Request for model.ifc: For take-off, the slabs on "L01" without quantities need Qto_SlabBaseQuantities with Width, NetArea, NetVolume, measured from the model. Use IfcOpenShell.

First a look at what the model holds.

```python
import ifcopenshell
import ifcopenshell.util.element
import ifcopenshell.util.unit

model = ifcopenshell.open("model.ifc")
print(model.schema)
for unit_type in ("LENGTHUNIT", "AREAUNIT", "VOLUMEUNIT"):
    print(unit_type, ifcopenshell.util.unit.calculate_unit_scale(model, unit_type))
storey = next(s for s in model.by_type("IfcBuildingStorey") if s.Name == "L01")
slabs = [e for e in ifcopenshell.util.element.get_decomposition(storey) if e.is_a("IfcSlab")]
for e in sorted(slabs, key=lambda e: e.id()):
    print(e.id(), e.is_a(), e.Name, list(ifcopenshell.util.element.get_psets(e, qtos_only=True)), sep=" | ")
```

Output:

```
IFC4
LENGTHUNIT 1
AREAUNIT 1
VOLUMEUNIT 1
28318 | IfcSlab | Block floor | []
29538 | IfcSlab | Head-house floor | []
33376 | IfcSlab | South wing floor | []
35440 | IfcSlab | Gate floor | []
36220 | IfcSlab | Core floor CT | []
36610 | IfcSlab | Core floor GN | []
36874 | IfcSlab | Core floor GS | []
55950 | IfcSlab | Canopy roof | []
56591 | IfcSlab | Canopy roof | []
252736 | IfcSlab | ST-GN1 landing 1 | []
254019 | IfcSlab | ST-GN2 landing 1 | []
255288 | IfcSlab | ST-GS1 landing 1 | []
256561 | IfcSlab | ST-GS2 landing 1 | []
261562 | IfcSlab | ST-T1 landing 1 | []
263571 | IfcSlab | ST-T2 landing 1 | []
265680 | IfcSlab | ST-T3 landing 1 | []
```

```python
import ifcopenshell
import ifcopenshell.api.pset
import ifcopenshell.geom
import ifcopenshell.util.element
import ifcopenshell.util.shape
import ifcopenshell.util.unit

model = ifcopenshell.open("model.ifc")
unit_scale = ifcopenshell.util.unit.calculate_unit_scale(model)
area_scale = ifcopenshell.util.unit.calculate_unit_scale(model, "AREAUNIT")
volume_scale = ifcopenshell.util.unit.calculate_unit_scale(model, "VOLUMEUNIT")
settings = ifcopenshell.geom.settings()

storey = next(s for s in model.by_type("IfcBuildingStorey") if s.Name == "L01")
slabs = [e for e in ifcopenshell.util.element.get_decomposition(storey) if e.is_a("IfcSlab")]

for e in sorted(slabs, key=lambda e: e.id()):
    if ifcopenshell.util.element.get_psets(e, qtos_only=True, should_inherit=False):
        continue
    # Geometry comes back in metres, in the element's own axes.
    shape = ifcopenshell.geom.create_shape(settings, e)
    values = {
        "Width": ifcopenshell.util.shape.get_z(shape.geometry) / unit_scale,
        "NetArea": ifcopenshell.util.shape.get_footprint_area(shape.geometry) / area_scale,
        "NetVolume": ifcopenshell.util.shape.get_volume(shape.geometry) / volume_scale,
    }
    qto = ifcopenshell.api.pset.add_qto(model, product=e, name="Qto_SlabBaseQuantities")
    ifcopenshell.api.pset.edit_qto(model, qto=qto, properties=values)
    print(e.id(), {k: round(v, 3) for k, v in values.items()})

model.write("model_rev.ifc")
```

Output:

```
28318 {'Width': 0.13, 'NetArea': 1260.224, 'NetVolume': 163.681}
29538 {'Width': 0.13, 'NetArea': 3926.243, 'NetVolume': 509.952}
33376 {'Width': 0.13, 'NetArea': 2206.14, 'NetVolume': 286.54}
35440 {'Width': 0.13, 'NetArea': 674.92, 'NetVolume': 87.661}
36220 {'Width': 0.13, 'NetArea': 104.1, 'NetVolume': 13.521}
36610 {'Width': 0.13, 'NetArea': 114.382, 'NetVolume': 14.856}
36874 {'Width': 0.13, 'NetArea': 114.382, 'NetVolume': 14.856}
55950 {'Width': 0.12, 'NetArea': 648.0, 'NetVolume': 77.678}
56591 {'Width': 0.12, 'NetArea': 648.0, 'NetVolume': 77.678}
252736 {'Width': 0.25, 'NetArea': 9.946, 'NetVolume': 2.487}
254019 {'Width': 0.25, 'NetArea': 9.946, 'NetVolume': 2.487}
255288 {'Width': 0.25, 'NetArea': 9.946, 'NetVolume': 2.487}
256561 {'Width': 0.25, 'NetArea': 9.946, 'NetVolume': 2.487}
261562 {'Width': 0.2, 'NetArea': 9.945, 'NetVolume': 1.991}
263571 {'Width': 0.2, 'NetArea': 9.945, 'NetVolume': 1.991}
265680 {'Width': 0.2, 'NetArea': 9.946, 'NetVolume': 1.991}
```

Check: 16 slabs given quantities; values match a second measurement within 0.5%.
